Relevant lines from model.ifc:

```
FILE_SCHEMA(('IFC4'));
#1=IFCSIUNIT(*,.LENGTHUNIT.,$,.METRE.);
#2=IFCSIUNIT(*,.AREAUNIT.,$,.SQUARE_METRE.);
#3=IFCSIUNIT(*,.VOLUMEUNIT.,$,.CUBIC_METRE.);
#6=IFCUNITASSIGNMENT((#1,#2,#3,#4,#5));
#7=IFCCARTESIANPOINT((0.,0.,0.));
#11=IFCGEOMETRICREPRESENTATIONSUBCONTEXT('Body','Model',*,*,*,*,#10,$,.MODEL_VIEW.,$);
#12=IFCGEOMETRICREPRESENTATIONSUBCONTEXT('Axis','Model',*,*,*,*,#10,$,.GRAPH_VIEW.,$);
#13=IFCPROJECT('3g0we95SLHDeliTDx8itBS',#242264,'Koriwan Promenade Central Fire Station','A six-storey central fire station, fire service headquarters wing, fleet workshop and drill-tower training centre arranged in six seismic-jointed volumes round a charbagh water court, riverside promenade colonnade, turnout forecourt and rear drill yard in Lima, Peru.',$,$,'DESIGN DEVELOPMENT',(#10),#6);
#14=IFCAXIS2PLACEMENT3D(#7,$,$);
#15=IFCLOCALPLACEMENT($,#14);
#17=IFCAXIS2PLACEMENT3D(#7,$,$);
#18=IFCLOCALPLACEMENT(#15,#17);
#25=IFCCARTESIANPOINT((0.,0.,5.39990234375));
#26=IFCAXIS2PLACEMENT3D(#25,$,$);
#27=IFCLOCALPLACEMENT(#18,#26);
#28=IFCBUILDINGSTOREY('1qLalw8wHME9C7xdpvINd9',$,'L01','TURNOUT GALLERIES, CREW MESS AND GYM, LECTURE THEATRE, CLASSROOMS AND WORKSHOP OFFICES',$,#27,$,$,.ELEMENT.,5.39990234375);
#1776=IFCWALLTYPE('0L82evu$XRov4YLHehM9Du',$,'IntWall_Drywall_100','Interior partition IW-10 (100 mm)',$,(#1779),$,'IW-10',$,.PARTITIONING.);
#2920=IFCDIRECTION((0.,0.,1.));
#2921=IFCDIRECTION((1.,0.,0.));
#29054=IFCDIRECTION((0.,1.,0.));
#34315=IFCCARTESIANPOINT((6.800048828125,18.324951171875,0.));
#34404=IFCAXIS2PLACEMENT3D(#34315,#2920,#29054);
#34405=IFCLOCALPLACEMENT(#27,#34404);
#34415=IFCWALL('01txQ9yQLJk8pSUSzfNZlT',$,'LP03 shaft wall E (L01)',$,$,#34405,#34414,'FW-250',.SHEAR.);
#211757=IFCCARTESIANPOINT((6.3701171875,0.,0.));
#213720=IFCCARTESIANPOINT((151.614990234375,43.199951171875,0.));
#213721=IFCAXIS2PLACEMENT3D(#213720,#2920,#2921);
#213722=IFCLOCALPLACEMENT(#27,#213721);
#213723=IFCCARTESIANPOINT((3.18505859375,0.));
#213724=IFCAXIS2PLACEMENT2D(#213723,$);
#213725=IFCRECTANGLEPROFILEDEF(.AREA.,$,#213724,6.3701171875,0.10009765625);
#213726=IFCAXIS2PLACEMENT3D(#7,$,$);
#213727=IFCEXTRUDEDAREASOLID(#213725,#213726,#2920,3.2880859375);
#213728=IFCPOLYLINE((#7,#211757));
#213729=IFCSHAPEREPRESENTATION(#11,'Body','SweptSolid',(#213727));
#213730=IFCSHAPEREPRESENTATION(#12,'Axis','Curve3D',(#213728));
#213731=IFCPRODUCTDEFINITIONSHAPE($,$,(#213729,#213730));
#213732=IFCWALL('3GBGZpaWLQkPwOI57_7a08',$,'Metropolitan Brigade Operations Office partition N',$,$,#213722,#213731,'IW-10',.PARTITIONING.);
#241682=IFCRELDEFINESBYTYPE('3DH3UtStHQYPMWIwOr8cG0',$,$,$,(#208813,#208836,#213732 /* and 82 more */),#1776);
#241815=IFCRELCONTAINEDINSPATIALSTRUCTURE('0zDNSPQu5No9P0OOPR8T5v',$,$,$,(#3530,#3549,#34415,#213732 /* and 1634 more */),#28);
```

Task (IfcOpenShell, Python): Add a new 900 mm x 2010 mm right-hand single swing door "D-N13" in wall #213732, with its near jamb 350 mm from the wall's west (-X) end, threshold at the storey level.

```python
import numpy as np
import ifcopenshell
import ifcopenshell.api.feature
import ifcopenshell.api.geometry
import ifcopenshell.api.root
import ifcopenshell.api.spatial
import ifcopenshell.geom
import ifcopenshell.util.element
import ifcopenshell.util.placement
import ifcopenshell.util.representation
import ifcopenshell.util.shape
import ifcopenshell.util.unit

model = ifcopenshell.open("model.ifc")
unit_scale = ifcopenshell.util.unit.calculate_unit_scale(model)
settings = ifcopenshell.geom.settings()


def volume(element):
    """Net volume in cubic metres, openings subtracted."""
    shape = ifcopenshell.geom.create_shape(settings, element)
    return ifcopenshell.util.shape.get_volume(shape.geometry)


wall = model.by_guid("3GBGZpaWLQkPwOI57_7a08")
storey = ifcopenshell.util.element.get_container(wall, ifc_class="IfcBuildingStorey")
context = ifcopenshell.util.representation.get_context(model, "Model", "Body", "MODEL_VIEW")
before = volume(wall)

width, height, from_end, sill = 0.9, 2.01, 0.35, 0.0  # metres

# The wall runs along its own X axis, and the end named is its -X end.
wall_shape = ifcopenshell.geom.create_shape(settings, wall)
x, y, z = ifcopenshell.util.shape.get_vertices(wall_shape.geometry).T
start = x.min() + from_end
face, thickness = float(y.min()), float(y.max() - y.min())
wall_matrix = ifcopenshell.util.placement.get_local_placement(wall.ObjectPlacement)
level = ifcopenshell.util.placement.get_local_placement(storey.ObjectPlacement)[2, 3]


def in_wall(x, y):
    """Placement at x, y metres in the wall's axes, at sill height."""
    matrix = wall_matrix.copy()
    matrix[:, 3] = wall_matrix @ np.array([x / unit_scale, y / unit_scale, 0.0, 1.0])
    matrix[2, 3] = level + sill / unit_scale
    return matrix


# Opening: a box that overshoots both wall faces by 50 mm.
opening = ifcopenshell.api.root.create_entity(model, ifc_class="IfcOpeningElement", predefined_type="OPENING")
box = ifcopenshell.api.geometry.add_wall_representation(
    model, context=context, length=width, height=height, thickness=thickness + 0.1
)
ifcopenshell.api.geometry.assign_representation(model, product=opening, representation=box)
ifcopenshell.api.geometry.edit_object_placement(model, product=opening, matrix=in_wall(start, face - 0.05), is_si=False)
ifcopenshell.api.feature.add_feature(model, feature=opening, element=wall)

door = ifcopenshell.api.root.create_entity(model, ifc_class="IfcDoor", name="D-N13", predefined_type="DOOR")
door.OverallWidth, door.OverallHeight = width / unit_scale, height / unit_scale
door.OperationType = "SINGLE_SWING_RIGHT"
body = ifcopenshell.api.geometry.add_door_representation(
    model,
    context=context,
    overall_width=door.OverallWidth,
    overall_height=door.OverallHeight,
    operation_type="SINGLE_SWING_RIGHT",
    lining_properties={"LiningDepth": thickness / unit_scale, "ThresholdDepth": thickness / unit_scale},
)
ifcopenshell.api.geometry.assign_representation(model, product=door, representation=body)
ifcopenshell.api.spatial.assign_container(model, products=[door], relating_structure=storey)
ifcopenshell.api.feature.add_filling(model, opening=opening, element=door)

# The lining spans the wall, so the door starts at the wall face.
ifcopenshell.api.geometry.edit_object_placement(model, product=door, matrix=in_wall(start, face), is_si=False)

after = volume(wall)

print(f"wall volume {before:.3f} -> {after:.3f} m3")

model.write("model_rev.ifc")
```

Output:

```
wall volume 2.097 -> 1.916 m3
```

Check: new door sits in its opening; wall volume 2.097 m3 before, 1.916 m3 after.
